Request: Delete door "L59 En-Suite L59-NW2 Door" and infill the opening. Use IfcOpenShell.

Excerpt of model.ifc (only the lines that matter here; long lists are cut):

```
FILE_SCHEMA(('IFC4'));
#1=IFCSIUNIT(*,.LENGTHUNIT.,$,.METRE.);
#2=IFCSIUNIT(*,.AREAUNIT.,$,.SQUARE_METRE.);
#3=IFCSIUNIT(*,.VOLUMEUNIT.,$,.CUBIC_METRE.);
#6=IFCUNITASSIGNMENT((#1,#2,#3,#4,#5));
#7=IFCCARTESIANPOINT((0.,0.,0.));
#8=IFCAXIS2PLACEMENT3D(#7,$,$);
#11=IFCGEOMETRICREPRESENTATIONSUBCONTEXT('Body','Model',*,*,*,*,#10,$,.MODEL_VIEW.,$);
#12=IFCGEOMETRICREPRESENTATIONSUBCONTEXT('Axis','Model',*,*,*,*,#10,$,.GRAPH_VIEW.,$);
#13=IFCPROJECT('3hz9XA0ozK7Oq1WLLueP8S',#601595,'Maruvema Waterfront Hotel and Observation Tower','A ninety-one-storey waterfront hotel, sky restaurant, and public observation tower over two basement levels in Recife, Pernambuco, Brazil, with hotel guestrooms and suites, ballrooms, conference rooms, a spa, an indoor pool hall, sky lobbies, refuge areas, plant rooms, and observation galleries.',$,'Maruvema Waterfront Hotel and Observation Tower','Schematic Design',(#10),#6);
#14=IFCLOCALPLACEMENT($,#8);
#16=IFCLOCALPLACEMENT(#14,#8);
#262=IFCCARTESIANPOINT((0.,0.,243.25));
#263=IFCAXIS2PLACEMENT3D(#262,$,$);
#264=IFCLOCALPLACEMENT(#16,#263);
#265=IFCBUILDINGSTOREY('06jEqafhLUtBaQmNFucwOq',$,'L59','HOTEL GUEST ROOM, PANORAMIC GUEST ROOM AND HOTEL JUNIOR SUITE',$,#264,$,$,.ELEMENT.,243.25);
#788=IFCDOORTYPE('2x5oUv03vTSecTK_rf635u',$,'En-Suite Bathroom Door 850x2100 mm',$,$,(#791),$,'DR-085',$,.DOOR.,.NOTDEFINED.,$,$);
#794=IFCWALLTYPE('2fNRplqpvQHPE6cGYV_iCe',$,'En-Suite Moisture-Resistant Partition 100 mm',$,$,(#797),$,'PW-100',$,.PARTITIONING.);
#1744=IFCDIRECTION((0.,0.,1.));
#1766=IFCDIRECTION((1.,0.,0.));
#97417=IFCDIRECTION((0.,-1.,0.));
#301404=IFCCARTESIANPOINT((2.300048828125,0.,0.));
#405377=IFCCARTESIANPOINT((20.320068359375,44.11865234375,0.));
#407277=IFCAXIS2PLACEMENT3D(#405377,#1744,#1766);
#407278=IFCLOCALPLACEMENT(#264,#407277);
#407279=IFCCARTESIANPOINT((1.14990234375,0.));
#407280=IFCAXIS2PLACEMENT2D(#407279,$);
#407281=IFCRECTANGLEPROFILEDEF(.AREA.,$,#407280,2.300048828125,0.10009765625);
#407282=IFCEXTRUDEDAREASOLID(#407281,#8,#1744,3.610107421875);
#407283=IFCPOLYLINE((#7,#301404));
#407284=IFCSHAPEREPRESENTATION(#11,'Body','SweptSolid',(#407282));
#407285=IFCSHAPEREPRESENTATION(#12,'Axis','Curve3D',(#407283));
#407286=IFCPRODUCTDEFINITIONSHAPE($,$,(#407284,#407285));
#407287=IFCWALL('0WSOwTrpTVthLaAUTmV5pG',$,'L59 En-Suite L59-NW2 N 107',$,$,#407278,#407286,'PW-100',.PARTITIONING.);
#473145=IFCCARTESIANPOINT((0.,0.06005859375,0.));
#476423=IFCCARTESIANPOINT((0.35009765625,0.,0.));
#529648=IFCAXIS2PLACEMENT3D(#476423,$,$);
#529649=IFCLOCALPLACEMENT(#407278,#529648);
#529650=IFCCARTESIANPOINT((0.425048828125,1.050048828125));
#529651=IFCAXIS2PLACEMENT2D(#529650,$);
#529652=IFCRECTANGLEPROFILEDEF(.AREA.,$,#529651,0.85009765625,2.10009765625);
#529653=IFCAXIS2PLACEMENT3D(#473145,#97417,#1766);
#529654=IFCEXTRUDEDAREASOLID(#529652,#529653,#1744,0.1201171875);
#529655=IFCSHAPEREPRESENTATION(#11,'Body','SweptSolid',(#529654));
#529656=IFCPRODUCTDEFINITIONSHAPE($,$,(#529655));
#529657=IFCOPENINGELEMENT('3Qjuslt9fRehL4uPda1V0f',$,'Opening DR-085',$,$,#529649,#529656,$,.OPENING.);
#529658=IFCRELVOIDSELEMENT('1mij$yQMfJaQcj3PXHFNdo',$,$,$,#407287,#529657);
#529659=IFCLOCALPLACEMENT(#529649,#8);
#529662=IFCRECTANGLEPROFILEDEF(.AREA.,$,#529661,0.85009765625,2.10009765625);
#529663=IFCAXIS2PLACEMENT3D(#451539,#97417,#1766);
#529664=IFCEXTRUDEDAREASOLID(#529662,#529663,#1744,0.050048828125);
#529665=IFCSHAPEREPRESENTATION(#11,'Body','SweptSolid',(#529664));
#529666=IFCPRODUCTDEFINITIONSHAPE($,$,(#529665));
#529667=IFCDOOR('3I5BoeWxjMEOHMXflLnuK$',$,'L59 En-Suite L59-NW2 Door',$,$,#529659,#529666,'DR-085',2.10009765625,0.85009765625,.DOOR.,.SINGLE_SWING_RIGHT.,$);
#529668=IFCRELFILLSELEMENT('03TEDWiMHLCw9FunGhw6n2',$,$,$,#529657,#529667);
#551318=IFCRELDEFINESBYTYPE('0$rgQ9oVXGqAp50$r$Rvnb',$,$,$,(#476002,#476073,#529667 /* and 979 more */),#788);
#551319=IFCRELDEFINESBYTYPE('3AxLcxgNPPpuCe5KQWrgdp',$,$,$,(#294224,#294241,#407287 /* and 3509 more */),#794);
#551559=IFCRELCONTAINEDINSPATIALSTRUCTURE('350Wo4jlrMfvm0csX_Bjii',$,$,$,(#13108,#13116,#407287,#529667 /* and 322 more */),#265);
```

```python
import ifcopenshell
import ifcopenshell.api.feature
import ifcopenshell.api.root
import ifcopenshell.geom
import ifcopenshell.util.shape

model = ifcopenshell.open("model.ifc")
settings = ifcopenshell.geom.settings()


def volume(element):
    """Net volume in cubic metres, openings subtracted."""
    shape = ifcopenshell.geom.create_shape(settings, element)
    return ifcopenshell.util.shape.get_volume(shape.geometry)


door = model.by_id(529667)
opening = door.FillsVoids[0].RelatingOpeningElement
wall = opening.VoidsElements[0].RelatingBuildingElement
before = volume(wall)

ifcopenshell.api.root.remove_product(model, product=door)
ifcopenshell.api.feature.remove_feature(model, feature=opening)

after = volume(wall)

print(f"wall volume {before:.3f} -> {after:.3f} m3")

model.write("model-out.ifc")
```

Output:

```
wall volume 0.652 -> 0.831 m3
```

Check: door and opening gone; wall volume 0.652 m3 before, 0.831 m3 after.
